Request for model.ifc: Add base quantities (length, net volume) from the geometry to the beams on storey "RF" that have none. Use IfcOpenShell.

First a look at what the model holds.

```python
import ifcopenshell
import ifcopenshell.util.element
import ifcopenshell.util.unit

model = ifcopenshell.open("model.ifc")
print(model.schema)
for unit_type in ("LENGTHUNIT", "AREAUNIT", "VOLUMEUNIT"):
    print(unit_type, ifcopenshell.util.unit.calculate_unit_scale(model, unit_type))
storey = next(s for s in model.by_type("IfcBuildingStorey") if s.Name == "RF")
beams = [e for e in ifcopenshell.util.element.get_decomposition(storey) if e.is_a("IfcBeam")]
for e in sorted(beams, key=lambda e: e.id()):
    print(e.id(), e.is_a(), e.Name, list(ifcopenshell.util.element.get_psets(e, qtos_only=True)), sep=" | ")
```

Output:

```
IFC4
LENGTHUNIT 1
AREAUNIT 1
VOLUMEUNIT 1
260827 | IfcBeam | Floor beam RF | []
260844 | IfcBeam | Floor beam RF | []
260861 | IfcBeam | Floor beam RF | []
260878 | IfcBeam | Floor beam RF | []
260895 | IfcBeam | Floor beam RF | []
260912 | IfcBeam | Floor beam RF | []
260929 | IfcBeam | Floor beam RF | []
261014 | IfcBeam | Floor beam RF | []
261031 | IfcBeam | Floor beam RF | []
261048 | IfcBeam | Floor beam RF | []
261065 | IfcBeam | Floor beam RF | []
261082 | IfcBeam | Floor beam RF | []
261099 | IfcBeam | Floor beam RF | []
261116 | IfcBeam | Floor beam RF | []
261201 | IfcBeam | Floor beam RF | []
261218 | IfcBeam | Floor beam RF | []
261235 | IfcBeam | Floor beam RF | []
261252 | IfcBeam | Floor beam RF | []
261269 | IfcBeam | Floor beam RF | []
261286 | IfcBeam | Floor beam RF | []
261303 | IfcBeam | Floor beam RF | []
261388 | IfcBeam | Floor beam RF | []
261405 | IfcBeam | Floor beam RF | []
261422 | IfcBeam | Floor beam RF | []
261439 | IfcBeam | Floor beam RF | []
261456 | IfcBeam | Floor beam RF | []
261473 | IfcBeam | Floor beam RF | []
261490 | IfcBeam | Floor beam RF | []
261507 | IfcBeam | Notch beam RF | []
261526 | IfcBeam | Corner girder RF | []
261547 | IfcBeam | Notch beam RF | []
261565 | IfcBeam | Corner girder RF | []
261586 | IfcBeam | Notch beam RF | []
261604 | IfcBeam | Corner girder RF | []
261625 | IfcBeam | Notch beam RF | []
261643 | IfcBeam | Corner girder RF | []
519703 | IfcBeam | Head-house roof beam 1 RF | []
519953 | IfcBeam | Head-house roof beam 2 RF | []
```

```python
import ifcopenshell
import ifcopenshell.api.pset
import ifcopenshell.geom
import ifcopenshell.util.element
import ifcopenshell.util.shape
import ifcopenshell.util.unit

model = ifcopenshell.open("model.ifc")
unit_scale = ifcopenshell.util.unit.calculate_unit_scale(model)
volume_scale = ifcopenshell.util.unit.calculate_unit_scale(model, "VOLUMEUNIT")
settings = ifcopenshell.geom.settings()

storey = next(s for s in model.by_type("IfcBuildingStorey") if s.Name == "RF")
beams = [e for e in ifcopenshell.util.element.get_decomposition(storey) if e.is_a("IfcBeam")]

for e in sorted(beams, key=lambda e: e.id()):
    if ifcopenshell.util.element.get_psets(e, qtos_only=True, should_inherit=False):
        continue
    # Geometry comes back in metres, in the element's own axes.
    shape = ifcopenshell.geom.create_shape(settings, e)
    values = {
        "Length": ifcopenshell.util.shape.get_max_xyz(shape.geometry) / unit_scale,
        "NetVolume": ifcopenshell.util.shape.get_volume(shape.geometry) / volume_scale,
    }
    qto = ifcopenshell.api.pset.add_qto(model, product=e, name="Qto_BeamBaseQuantities")
    ifcopenshell.api.pset.edit_qto(model, qto=qto, properties=values)
    print(e.id(), {k: round(v, 3) for k, v in values.items()})

model.write("model_updated.ifc")
```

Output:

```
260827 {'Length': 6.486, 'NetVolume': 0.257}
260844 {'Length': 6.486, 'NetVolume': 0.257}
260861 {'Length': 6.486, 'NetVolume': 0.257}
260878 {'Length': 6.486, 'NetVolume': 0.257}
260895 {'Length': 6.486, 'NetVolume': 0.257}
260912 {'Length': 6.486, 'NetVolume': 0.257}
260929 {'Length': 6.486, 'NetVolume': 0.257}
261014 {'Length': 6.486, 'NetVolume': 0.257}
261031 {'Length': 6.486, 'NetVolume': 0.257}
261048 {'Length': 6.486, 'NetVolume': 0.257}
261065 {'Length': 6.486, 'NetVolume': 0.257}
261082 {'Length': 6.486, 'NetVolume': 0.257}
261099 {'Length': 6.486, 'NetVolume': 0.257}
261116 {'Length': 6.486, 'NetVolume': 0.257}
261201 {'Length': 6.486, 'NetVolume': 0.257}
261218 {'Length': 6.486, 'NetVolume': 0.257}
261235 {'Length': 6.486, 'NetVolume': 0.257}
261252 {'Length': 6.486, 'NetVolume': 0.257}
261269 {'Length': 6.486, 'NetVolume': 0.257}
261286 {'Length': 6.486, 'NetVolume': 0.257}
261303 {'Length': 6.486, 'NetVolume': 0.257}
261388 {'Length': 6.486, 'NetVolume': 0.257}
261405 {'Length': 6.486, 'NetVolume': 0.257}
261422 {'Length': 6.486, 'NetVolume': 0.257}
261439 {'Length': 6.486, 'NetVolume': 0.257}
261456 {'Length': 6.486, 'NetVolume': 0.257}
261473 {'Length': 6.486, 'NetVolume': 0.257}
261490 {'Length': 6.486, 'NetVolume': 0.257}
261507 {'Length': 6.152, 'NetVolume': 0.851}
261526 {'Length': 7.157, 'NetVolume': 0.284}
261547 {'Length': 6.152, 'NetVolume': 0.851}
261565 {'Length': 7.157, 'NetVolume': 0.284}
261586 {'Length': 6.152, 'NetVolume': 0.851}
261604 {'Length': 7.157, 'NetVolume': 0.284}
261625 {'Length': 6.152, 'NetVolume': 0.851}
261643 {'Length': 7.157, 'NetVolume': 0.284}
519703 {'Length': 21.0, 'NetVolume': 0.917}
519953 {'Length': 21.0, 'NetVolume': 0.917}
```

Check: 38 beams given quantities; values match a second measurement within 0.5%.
